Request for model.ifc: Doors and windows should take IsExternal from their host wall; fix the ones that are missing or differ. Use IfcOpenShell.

First a look at what the model holds.

```python
import ifcopenshell
import ifcopenshell.util.element

model = ifcopenshell.open("model.ifc")
print(model.schema)
seen = {}
for e in model.by_type("IfcDoor") + model.by_type("IfcWindow"):
    if not e.FillsVoids:
        continue
    host = e.FillsVoids[0].RelatingOpeningElement.VoidsElements[0].RelatingBuildingElement
    own = ifcopenshell.util.element.get_pset(e, f"Pset_{e.is_a()[3:].removesuffix('StandardCase')}Common", "IsExternal")
    wall = ifcopenshell.util.element.get_pset(host, "Pset_WallCommon", "IsExternal")
    seen[e.is_a(), own, wall] = seen.get((e.is_a(), own, wall), 0) + 1
for (cls, own, wall), count in sorted(seen.items(), key=str):
    print(count, cls, "IsExternal:", own, "| host wall:", wall)
```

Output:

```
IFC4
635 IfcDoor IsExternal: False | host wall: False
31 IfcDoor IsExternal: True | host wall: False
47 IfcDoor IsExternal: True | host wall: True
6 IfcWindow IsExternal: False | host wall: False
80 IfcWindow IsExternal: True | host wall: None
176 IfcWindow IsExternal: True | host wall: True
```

```python
import ifcopenshell
import ifcopenshell.api.pset
import ifcopenshell.util.element

model = ifcopenshell.open("model.ifc")

count = 0
for ifc_class, pset_name in (("IfcDoor", "Pset_DoorCommon"), ("IfcWindow", "Pset_WindowCommon")):
    for e in model.by_type(ifc_class):
        if not e.FillsVoids:
            continue
        host = e.FillsVoids[0].RelatingOpeningElement.VoidsElements[0].RelatingBuildingElement
        external = ifcopenshell.util.element.get_pset(host, "Pset_WallCommon", "IsExternal")
        if external is None or ifcopenshell.util.element.get_pset(e, pset_name, "IsExternal") == external:
            continue
        pset = ifcopenshell.api.pset.add_pset(model, product=e, name=pset_name)
        ifcopenshell.api.pset.edit_pset(model, pset=pset, properties={"IsExternal": external})
        count += 1

print(count, "updated")

model.write("model_updated.ifc")
```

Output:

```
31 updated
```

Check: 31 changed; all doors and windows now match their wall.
